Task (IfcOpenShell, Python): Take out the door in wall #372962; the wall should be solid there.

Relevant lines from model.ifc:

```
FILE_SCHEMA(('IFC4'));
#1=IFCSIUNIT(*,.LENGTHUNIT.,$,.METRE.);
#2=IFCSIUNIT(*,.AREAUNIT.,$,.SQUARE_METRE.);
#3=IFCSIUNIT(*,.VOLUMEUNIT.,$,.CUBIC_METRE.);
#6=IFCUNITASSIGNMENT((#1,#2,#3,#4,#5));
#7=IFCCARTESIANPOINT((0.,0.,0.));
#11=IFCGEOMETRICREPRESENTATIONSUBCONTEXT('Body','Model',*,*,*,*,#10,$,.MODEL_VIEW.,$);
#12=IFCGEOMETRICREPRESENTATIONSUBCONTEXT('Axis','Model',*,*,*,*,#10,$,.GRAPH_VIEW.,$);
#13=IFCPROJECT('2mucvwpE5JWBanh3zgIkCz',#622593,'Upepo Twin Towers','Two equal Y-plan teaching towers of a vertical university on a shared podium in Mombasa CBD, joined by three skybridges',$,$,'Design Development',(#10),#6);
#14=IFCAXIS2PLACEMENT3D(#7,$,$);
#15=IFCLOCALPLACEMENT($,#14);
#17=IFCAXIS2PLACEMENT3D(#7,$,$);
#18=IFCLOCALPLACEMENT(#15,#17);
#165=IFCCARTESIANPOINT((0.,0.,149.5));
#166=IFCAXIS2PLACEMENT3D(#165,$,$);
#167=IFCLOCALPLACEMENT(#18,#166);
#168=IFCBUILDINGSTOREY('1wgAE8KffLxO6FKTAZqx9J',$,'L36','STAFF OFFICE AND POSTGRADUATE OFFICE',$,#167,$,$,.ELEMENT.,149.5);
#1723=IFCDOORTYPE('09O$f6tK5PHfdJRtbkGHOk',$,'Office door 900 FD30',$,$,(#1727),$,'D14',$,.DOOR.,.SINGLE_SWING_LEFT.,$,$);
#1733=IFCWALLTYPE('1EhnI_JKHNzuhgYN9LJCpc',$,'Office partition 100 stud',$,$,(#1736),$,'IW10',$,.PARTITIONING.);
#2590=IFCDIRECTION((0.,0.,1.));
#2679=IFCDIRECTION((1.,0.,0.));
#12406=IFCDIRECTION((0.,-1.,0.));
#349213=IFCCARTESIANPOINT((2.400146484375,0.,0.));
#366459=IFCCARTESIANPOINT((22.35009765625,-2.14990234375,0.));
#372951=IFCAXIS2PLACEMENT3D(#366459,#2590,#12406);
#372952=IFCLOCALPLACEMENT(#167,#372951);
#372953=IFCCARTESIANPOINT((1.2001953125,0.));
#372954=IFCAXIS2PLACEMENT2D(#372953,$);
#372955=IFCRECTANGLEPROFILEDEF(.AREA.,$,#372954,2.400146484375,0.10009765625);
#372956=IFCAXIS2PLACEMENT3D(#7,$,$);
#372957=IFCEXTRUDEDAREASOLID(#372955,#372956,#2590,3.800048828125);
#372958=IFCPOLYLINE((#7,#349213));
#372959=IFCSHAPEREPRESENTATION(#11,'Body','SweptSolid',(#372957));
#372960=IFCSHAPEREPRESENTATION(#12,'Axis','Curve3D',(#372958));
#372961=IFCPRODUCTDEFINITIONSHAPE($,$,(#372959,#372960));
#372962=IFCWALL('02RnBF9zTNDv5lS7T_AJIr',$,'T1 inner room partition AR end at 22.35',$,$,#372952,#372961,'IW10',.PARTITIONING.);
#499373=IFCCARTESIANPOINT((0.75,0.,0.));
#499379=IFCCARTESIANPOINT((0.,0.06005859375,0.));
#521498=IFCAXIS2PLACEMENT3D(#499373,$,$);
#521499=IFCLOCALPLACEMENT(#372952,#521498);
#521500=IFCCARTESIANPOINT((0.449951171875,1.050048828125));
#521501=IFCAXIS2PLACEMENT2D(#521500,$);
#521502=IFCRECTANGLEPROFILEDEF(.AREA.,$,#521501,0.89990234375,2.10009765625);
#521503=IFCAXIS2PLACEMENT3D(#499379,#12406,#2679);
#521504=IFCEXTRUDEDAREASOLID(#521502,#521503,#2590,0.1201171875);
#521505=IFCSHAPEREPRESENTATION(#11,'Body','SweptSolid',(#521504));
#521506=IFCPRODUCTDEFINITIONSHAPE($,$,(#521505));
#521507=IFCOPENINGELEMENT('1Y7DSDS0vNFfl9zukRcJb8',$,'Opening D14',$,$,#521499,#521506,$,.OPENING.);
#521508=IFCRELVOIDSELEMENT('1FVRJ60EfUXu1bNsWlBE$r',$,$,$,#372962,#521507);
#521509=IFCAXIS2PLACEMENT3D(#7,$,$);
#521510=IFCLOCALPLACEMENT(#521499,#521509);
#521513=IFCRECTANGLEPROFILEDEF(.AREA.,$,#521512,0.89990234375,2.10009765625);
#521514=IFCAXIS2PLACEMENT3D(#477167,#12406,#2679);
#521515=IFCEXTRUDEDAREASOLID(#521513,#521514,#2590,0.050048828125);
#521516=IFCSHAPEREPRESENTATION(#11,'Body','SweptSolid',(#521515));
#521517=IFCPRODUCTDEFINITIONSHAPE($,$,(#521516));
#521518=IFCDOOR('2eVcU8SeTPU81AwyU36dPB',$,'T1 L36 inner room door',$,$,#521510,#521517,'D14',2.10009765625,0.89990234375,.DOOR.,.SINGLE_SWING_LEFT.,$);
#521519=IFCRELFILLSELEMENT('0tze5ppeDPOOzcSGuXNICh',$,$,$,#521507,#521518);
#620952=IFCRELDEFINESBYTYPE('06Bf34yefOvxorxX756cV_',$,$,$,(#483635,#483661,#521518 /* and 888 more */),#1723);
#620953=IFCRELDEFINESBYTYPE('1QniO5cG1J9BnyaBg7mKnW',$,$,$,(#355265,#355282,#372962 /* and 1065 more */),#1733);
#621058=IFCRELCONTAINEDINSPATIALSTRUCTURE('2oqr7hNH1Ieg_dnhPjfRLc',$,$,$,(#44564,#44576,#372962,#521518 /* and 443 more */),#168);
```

```python
import ifcopenshell
import ifcopenshell.api.feature
import ifcopenshell.api.root
import ifcopenshell.geom
import ifcopenshell.util.shape

model = ifcopenshell.open("model.ifc")
settings = ifcopenshell.geom.settings()


def volume(element):
    """Net volume in cubic metres, openings subtracted."""
    shape = ifcopenshell.geom.create_shape(settings, element)
    return ifcopenshell.util.shape.get_volume(shape.geometry)


door = model.by_id(521518)
opening = door.FillsVoids[0].RelatingOpeningElement
wall = opening.VoidsElements[0].RelatingBuildingElement
before = volume(wall)

ifcopenshell.api.root.remove_product(model, product=door)
ifcopenshell.api.feature.remove_feature(model, feature=opening)

after = volume(wall)

print(f"wall volume {before:.3f} -> {after:.3f} m3")

model.write("model_updated.ifc")
```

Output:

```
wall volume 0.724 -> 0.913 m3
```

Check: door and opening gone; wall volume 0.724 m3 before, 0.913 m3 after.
